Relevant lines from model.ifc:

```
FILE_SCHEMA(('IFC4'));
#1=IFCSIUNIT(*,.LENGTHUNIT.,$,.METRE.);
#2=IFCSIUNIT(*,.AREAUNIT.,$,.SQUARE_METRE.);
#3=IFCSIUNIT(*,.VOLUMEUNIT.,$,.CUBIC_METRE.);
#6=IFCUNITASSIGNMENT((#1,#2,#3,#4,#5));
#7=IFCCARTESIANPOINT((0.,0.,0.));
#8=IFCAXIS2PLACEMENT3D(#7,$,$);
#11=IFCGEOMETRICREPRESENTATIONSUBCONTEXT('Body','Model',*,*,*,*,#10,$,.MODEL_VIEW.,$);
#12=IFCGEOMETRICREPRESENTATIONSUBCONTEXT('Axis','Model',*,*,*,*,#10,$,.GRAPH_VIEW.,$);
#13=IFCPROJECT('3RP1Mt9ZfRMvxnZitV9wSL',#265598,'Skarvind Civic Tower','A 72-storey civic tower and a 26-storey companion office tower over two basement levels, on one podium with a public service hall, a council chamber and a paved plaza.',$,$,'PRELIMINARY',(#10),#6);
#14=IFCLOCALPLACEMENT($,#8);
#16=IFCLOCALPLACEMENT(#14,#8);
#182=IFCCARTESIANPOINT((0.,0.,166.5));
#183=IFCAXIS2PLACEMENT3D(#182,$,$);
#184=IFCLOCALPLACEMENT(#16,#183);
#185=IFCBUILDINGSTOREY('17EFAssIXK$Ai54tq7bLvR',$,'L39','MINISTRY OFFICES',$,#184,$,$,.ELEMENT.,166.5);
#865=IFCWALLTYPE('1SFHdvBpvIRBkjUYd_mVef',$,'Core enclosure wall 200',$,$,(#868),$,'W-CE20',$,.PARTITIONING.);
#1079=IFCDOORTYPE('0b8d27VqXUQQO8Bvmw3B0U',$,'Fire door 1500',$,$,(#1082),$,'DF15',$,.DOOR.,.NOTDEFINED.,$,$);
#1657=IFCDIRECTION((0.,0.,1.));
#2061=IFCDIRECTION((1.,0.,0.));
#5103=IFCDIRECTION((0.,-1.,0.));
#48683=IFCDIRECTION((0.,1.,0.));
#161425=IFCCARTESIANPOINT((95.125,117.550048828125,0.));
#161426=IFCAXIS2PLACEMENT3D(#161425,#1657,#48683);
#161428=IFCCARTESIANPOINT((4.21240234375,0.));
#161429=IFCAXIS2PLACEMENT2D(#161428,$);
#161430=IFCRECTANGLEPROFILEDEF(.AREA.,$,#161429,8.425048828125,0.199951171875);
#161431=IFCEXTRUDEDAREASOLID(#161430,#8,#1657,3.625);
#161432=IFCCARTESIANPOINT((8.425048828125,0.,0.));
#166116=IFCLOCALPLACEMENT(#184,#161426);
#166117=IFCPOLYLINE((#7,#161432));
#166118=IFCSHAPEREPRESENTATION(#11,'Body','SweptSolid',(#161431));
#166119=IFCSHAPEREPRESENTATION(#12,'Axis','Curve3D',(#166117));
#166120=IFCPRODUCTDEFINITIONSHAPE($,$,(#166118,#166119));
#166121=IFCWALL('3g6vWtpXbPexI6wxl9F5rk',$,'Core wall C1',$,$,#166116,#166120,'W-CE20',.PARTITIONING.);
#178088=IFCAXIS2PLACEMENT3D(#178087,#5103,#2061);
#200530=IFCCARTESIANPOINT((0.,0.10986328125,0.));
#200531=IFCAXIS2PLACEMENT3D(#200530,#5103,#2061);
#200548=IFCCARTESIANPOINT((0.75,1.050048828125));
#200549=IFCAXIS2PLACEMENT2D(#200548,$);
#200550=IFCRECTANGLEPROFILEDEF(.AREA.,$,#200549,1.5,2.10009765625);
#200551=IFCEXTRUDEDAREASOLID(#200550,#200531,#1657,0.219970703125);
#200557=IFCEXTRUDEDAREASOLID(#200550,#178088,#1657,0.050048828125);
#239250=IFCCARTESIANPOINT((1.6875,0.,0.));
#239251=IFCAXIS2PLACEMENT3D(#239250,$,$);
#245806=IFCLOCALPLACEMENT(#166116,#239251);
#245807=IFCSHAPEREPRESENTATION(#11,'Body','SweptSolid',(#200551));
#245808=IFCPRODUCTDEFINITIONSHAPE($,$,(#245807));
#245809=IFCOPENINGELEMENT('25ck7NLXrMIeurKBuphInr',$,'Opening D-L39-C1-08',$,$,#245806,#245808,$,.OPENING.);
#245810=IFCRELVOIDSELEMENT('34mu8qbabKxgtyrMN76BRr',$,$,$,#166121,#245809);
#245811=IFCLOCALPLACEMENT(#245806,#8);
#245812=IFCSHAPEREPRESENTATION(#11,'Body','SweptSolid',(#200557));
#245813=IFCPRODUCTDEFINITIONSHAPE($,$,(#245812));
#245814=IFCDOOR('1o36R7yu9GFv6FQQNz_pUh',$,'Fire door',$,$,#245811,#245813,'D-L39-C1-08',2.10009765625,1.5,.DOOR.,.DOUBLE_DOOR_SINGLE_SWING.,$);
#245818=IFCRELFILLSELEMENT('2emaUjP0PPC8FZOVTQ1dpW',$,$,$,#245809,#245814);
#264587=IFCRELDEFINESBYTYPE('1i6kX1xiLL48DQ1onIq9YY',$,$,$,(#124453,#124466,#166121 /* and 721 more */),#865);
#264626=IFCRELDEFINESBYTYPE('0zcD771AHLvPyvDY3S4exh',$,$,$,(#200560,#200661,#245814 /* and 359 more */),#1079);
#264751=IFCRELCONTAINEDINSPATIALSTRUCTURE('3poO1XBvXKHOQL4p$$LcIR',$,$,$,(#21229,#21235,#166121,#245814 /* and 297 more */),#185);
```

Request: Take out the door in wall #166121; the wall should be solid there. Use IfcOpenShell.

```python
import ifcopenshell
import ifcopenshell.api.feature
import ifcopenshell.api.root
import ifcopenshell.geom
import ifcopenshell.util.shape

model = ifcopenshell.open("model.ifc")
settings = ifcopenshell.geom.settings()


def volume(element):
    """Net volume in cubic metres, openings subtracted."""
    shape = ifcopenshell.geom.create_shape(settings, element)
    return ifcopenshell.util.shape.get_volume(shape.geometry)


door = model.by_id(245814)
opening = door.FillsVoids[0].RelatingOpeningElement
wall = opening.VoidsElements[0].RelatingBuildingElement
before = volume(wall)

ifcopenshell.api.root.remove_product(model, product=door)
ifcopenshell.api.feature.remove_feature(model, feature=opening)

after = volume(wall)

print(f"wall volume {before:.3f} -> {after:.3f} m3")

model.write("model_rev.ifc")
```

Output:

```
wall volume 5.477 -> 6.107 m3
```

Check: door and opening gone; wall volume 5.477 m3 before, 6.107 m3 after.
